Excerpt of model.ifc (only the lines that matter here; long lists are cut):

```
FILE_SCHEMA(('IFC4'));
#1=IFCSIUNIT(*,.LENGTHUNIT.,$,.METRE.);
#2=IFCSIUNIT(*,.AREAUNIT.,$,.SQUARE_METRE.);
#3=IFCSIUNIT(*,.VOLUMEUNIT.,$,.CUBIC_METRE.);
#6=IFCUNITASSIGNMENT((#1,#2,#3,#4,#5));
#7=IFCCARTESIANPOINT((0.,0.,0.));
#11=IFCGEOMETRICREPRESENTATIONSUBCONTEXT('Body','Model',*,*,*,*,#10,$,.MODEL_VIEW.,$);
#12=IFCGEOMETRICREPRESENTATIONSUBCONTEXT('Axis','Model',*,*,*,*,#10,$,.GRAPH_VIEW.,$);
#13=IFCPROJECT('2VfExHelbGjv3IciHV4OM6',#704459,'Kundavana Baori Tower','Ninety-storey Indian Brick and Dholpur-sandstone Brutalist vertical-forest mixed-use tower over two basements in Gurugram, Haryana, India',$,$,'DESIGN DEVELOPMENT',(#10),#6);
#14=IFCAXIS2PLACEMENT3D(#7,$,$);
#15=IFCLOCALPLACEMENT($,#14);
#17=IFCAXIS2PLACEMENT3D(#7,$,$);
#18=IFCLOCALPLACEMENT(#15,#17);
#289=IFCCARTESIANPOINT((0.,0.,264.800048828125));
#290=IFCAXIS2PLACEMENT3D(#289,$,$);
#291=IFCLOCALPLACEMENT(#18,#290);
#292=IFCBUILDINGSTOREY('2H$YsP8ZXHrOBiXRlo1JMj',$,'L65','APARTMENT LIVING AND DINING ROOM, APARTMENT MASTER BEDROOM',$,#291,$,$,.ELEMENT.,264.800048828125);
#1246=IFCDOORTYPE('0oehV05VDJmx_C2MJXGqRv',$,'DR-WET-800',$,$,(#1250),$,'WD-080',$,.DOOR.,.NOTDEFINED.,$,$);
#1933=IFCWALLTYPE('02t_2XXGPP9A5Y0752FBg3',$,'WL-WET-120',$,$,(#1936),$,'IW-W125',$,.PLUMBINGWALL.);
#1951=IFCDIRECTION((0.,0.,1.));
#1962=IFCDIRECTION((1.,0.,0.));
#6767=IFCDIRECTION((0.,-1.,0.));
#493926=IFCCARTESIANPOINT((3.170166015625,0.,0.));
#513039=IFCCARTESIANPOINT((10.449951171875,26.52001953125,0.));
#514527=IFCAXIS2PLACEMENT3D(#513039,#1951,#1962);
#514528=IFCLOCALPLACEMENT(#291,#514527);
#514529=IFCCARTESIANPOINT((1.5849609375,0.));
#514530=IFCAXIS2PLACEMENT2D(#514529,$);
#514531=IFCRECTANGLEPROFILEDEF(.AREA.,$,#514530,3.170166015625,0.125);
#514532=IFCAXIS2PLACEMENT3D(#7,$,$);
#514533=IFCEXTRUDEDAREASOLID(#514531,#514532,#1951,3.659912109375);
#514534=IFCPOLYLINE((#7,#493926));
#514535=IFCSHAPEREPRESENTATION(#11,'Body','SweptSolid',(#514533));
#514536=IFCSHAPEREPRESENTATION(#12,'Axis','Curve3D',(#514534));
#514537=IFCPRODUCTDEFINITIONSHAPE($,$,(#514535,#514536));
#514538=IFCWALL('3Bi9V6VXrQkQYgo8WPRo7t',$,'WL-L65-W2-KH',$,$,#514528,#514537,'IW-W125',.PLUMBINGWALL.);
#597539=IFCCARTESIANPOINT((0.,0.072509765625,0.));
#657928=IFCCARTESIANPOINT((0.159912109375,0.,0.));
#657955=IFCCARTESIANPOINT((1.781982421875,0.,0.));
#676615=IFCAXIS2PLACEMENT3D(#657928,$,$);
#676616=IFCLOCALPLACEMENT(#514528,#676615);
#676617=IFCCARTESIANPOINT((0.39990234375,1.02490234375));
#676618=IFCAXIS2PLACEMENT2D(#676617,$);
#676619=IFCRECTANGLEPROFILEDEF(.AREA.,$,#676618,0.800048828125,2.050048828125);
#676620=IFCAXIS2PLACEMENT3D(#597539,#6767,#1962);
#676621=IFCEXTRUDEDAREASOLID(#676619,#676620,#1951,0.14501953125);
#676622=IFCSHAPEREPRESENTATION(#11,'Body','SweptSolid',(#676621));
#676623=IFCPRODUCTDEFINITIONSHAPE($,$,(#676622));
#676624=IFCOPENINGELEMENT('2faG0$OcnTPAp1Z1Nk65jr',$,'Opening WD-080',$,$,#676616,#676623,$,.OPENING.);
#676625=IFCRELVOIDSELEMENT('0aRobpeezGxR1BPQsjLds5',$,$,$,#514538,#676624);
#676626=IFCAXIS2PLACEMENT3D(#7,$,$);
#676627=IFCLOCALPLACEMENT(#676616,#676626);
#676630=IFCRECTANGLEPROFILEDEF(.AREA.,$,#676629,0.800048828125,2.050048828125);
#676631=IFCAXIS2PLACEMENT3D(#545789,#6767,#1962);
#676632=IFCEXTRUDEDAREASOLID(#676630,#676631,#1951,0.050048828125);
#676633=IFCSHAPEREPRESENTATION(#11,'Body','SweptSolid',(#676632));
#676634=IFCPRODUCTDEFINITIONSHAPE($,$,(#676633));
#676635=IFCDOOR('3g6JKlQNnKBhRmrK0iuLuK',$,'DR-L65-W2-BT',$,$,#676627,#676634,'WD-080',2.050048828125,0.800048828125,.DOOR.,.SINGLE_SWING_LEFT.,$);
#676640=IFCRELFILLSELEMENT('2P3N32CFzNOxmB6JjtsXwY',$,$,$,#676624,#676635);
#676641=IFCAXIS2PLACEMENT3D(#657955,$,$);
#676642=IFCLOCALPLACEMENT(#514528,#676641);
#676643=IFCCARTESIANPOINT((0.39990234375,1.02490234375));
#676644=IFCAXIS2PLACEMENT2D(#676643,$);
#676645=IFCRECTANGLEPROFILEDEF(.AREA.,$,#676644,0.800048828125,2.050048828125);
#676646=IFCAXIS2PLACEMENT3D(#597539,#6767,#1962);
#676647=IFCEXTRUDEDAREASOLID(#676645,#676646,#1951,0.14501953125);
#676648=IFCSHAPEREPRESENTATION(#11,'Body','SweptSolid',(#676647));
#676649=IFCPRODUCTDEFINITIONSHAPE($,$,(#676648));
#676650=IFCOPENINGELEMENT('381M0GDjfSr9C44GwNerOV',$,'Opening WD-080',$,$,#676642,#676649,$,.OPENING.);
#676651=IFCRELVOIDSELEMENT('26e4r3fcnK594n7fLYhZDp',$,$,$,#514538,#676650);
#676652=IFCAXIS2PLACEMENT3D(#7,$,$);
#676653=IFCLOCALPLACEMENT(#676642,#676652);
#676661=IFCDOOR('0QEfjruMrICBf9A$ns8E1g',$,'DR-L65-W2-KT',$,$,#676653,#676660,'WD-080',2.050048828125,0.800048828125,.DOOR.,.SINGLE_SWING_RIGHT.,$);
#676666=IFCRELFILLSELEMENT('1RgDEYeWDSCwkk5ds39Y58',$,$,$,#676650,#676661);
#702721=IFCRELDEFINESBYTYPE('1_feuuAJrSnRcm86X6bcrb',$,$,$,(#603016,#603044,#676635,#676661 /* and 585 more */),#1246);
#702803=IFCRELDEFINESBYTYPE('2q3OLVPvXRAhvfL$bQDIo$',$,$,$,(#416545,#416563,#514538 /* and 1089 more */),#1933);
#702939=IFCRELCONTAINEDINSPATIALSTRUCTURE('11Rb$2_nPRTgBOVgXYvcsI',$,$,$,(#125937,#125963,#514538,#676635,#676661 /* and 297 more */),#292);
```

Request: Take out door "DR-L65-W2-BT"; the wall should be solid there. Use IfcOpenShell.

```python
import ifcopenshell
import ifcopenshell.api.feature
import ifcopenshell.api.root
import ifcopenshell.geom
import ifcopenshell.util.shape

model = ifcopenshell.open("model.ifc")
settings = ifcopenshell.geom.settings()


def volume(element):
    """Net volume in cubic metres, openings subtracted."""
    shape = ifcopenshell.geom.create_shape(settings, element)
    return ifcopenshell.util.shape.get_volume(shape.geometry)


door = model.by_guid("3g6JKlQNnKBhRmrK0iuLuK")
opening = door.FillsVoids[0].RelatingOpeningElement
wall = opening.VoidsElements[0].RelatingBuildingElement
before = volume(wall)

ifcopenshell.api.root.remove_product(model, product=door)
ifcopenshell.api.feature.remove_feature(model, feature=opening)

after = volume(wall)

print(f"wall volume {before:.3f} -> {after:.3f} m3")

model.write("model-out.ifc")
```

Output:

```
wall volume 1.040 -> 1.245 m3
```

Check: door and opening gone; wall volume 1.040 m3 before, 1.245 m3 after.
